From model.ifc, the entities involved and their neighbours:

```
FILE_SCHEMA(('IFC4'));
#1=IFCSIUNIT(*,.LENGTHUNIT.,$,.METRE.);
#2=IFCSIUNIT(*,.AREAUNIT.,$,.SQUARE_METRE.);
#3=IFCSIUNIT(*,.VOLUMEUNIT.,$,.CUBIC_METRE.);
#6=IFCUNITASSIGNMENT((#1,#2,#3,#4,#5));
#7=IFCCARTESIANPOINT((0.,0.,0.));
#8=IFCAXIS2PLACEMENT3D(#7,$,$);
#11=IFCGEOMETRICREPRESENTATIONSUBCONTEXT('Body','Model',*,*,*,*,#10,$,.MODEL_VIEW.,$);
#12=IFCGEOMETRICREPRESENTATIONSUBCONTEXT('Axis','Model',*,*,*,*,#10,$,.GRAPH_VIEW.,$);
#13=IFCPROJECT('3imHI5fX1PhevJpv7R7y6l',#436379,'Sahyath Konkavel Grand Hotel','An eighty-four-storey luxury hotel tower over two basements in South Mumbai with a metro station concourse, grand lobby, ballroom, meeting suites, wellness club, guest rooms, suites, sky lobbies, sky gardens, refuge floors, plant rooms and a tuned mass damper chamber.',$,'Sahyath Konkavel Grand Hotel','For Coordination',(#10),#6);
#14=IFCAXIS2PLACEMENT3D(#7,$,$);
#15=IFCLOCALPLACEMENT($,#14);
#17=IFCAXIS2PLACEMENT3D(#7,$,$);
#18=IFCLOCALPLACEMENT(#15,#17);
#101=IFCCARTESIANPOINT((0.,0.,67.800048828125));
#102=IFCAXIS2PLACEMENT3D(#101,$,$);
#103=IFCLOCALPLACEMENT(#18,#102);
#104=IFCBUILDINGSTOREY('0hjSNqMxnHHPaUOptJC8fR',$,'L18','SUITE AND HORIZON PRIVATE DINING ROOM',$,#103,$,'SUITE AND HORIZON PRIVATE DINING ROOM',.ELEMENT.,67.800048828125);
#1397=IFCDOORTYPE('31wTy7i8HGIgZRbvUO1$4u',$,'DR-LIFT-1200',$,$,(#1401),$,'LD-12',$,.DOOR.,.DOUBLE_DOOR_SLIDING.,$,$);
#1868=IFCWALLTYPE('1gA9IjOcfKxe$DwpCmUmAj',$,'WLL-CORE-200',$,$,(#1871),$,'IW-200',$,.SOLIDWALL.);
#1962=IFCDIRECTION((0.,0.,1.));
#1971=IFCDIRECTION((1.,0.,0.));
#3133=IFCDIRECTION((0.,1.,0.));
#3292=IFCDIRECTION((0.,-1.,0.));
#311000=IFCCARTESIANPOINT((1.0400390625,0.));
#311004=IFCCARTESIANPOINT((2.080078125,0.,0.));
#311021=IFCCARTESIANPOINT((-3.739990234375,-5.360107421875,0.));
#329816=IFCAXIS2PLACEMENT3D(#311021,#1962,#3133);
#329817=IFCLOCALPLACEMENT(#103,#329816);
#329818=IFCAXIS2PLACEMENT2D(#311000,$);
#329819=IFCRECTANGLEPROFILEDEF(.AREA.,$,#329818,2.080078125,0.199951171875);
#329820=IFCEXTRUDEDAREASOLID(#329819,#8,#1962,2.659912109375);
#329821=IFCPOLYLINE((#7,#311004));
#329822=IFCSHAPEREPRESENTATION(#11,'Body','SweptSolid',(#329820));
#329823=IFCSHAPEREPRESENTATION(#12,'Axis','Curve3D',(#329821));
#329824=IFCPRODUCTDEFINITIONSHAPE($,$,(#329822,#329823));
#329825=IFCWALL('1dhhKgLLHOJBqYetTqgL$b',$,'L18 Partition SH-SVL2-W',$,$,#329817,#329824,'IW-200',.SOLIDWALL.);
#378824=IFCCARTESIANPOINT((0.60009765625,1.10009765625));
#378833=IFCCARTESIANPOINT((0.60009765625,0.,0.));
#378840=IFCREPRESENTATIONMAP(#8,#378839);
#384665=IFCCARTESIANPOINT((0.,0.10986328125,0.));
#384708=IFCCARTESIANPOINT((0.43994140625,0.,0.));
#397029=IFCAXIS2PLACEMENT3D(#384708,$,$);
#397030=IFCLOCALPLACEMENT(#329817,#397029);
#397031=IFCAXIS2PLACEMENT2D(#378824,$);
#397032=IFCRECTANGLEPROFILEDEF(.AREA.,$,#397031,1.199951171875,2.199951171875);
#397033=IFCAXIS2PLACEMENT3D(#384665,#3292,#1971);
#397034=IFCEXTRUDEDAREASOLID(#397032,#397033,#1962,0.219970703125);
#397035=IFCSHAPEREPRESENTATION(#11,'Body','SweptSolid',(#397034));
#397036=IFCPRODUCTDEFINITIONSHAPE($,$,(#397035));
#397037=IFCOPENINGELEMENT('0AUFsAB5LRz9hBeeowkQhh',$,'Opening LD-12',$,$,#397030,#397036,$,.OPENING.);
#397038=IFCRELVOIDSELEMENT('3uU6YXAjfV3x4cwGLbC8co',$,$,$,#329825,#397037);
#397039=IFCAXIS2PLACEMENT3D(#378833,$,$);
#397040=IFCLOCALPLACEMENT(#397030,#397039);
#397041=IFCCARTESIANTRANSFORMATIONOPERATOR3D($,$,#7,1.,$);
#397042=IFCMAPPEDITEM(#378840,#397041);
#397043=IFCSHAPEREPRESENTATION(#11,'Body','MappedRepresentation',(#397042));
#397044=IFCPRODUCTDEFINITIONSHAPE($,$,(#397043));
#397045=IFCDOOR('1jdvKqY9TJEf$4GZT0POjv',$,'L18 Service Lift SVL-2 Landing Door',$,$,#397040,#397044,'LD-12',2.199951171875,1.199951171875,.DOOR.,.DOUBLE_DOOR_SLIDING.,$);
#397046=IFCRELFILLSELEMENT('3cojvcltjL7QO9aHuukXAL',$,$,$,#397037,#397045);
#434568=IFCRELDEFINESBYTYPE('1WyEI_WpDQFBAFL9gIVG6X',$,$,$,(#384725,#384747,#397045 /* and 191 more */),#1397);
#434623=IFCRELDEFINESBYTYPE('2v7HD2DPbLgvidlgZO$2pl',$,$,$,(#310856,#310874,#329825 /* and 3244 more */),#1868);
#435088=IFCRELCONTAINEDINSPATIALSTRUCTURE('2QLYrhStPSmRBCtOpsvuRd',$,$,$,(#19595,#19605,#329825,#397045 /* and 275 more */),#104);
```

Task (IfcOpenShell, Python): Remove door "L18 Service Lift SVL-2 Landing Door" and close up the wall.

```python
import ifcopenshell
import ifcopenshell.api.feature
import ifcopenshell.api.root
import ifcopenshell.geom
import ifcopenshell.util.shape

model = ifcopenshell.open("model.ifc")
settings = ifcopenshell.geom.settings()


def volume(element):
    """Net volume in cubic metres, openings subtracted."""
    shape = ifcopenshell.geom.create_shape(settings, element)
    return ifcopenshell.util.shape.get_volume(shape.geometry)


door = model.by_guid("1jdvKqY9TJEf$4GZT0POjv")
opening = door.FillsVoids[0].RelatingOpeningElement
wall = opening.VoidsElements[0].RelatingBuildingElement
before = volume(wall)

ifcopenshell.api.root.remove_product(model, product=door)
ifcopenshell.api.feature.remove_feature(model, feature=opening)

after = volume(wall)

print(f"wall volume {before:.3f} -> {after:.3f} m3")

model.write("model_updated.ifc")
```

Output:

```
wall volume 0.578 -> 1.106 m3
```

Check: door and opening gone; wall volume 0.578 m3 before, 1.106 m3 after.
